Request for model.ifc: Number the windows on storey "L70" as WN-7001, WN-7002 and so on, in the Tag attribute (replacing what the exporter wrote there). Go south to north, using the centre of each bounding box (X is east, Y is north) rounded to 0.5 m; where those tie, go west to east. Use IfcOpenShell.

First a look at what the model holds.

```python
import ifcopenshell
import ifcopenshell.util.element
import ifcopenshell.util.placement

model = ifcopenshell.open("model.ifc")
print(model.schema)
storey = next(s for s in model.by_type("IfcBuildingStorey") if s.Name == "L70")
windows = [e for e in ifcopenshell.util.element.get_decomposition(storey) if e.is_a("IfcWindow")]
for e in sorted(windows, key=lambda e: e.id()):
    origin = ifcopenshell.util.placement.get_local_placement(e.ObjectPlacement)[:3, 3]
    print(e.id(), e.Tag, e.Name, origin.round(2) + 0.0, sep=" | ")
```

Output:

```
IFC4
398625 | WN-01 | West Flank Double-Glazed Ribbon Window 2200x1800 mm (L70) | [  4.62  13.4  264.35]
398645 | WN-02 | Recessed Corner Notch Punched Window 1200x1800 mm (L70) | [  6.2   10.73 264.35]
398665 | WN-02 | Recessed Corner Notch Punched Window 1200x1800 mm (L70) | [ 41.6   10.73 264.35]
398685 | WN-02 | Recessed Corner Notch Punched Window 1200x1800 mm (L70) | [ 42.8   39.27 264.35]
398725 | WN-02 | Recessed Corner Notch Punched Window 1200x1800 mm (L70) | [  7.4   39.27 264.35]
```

```python
import ifcopenshell
import ifcopenshell.geom
import ifcopenshell.util.element
import ifcopenshell.util.shape

model = ifcopenshell.open("model.ifc")
settings = ifcopenshell.geom.settings()
settings.set("use-world-coords", True)


def centre(element):
    shape = ifcopenshell.geom.create_shape(settings, element)
    return ifcopenshell.util.shape.get_bbox_centroid(shape.geometry)


storey = next(s for s in model.by_type("IfcBuildingStorey") if s.Name == "L70")
windows = [e for e in ifcopenshell.util.element.get_decomposition(storey) if e.is_a("IfcWindow")]

# Insertion points can sit at a corner or the storey origin, so sort by the geometry (in metres).
centres = {e: centre(e) for e in windows}
windows.sort(key=lambda e: (round(centres[e][1] / 0.5), centres[e][0]))

for i, e in enumerate(windows, start=1):
    number = f"WN-70{i:02d}"
    e.Tag = number
    print(e.id(), number)

model.write("model_v2.ifc")
```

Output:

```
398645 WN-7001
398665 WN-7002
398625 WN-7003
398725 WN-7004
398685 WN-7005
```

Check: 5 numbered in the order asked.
